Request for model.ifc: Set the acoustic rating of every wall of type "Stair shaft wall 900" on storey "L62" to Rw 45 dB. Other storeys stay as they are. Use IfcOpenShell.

First a look at what the model holds.

```python
import ifcopenshell
import ifcopenshell.util.element

model = ifcopenshell.open("model.ifc")
print(model.schema)
storey = next(s for s in model.by_type("IfcBuildingStorey") if s.Name == "L62")
walls = [e for e in ifcopenshell.util.element.get_decomposition(storey) if e.is_a("IfcWall")]
seen = {}
for e in walls:
    element_type = ifcopenshell.util.element.get_type(e)
    key = (element_type.Name if element_type != e and element_type else None, ifcopenshell.util.element.get_pset(e, "Pset_WallCommon", "AcousticRating"))
    seen[key] = seen.get(key, 0) + 1
for (name, value), count in sorted(seen.items(), key=str):
    print(count, "x", name, "|", value)
```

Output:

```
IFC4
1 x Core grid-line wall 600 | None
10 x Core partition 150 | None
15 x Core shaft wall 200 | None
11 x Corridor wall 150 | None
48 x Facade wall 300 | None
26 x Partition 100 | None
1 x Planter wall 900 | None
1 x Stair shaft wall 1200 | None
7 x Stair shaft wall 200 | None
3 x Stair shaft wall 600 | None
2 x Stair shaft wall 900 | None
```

```python
import ifcopenshell
import ifcopenshell.api.pset
import ifcopenshell.util.element

model = ifcopenshell.open("model.ifc")

storey = next(s for s in model.by_type("IfcBuildingStorey") if s.Name == "L62")
walls = [e for e in ifcopenshell.util.element.get_decomposition(storey) if e.is_a("IfcWall")]

count = 0
for e in walls:
    element_type = ifcopenshell.util.element.get_type(e)
    if element_type in (None, e) or element_type.Name != "Stair shaft wall 900":
        continue
    # add_pset returns the element's existing set when there is one.
    pset = ifcopenshell.api.pset.add_pset(model, product=e, name="Pset_WallCommon")
    ifcopenshell.api.pset.edit_pset(model, pset=pset, properties={"AcousticRating": "Rw 45 dB"})
    count += 1

print(count, "walls updated")

model.write("model_edited.ifc")
```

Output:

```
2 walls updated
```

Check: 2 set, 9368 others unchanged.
